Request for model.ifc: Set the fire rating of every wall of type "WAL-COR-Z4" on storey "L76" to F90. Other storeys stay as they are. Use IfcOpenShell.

First a look at what the model holds.

```python
import ifcopenshell
import ifcopenshell.util.element

model = ifcopenshell.open("model.ifc")
print(model.schema)
storey = next(s for s in model.by_type("IfcBuildingStorey") if s.Name == "L76")
walls = [e for e in ifcopenshell.util.element.get_decomposition(storey) if e.is_a("IfcWall")]
seen = {}
for e in walls:
    element_type = ifcopenshell.util.element.get_type(e)
    key = (element_type.Name if element_type != e and element_type else None, ifcopenshell.util.element.get_pset(e, "Pset_WallCommon", "FireRating"))
    seen[key] = seen.get(key, 0) + 1
for (name, value), count in sorted(seen.items(), key=str):
    print(count, "x", name, "|", value)
```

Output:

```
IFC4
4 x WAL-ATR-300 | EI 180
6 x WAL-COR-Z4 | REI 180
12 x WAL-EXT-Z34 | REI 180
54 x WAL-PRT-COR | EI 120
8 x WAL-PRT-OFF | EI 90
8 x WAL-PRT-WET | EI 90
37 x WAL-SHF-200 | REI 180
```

```python
import ifcopenshell
import ifcopenshell.api.pset
import ifcopenshell.util.element

model = ifcopenshell.open("model.ifc")

storey = next(s for s in model.by_type("IfcBuildingStorey") if s.Name == "L76")
walls = [e for e in ifcopenshell.util.element.get_decomposition(storey) if e.is_a("IfcWall")]

count = 0
for e in walls:
    element_type = ifcopenshell.util.element.get_type(e)
    if element_type in (None, e) or element_type.Name != "WAL-COR-Z4":
        continue
    found = ifcopenshell.util.element.get_pset(e, "Pset_WallCommon", should_inherit=False)
    if found:
        pset = model.by_id(found["id"])
        if len(ifcopenshell.util.element.get_elements_by_pset(pset)) > 1:
            pset = ifcopenshell.api.pset.unshare_pset(model, products=[e], pset=pset)[0]
    else:
        pset = ifcopenshell.api.pset.add_pset(model, product=e, name="Pset_WallCommon")
    ifcopenshell.api.pset.edit_pset(model, pset=pset, properties={"FireRating": "F90"})
    count += 1

print(count, "walls updated")

model.write("model_edited.ifc")
```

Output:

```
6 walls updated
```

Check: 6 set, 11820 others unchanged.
